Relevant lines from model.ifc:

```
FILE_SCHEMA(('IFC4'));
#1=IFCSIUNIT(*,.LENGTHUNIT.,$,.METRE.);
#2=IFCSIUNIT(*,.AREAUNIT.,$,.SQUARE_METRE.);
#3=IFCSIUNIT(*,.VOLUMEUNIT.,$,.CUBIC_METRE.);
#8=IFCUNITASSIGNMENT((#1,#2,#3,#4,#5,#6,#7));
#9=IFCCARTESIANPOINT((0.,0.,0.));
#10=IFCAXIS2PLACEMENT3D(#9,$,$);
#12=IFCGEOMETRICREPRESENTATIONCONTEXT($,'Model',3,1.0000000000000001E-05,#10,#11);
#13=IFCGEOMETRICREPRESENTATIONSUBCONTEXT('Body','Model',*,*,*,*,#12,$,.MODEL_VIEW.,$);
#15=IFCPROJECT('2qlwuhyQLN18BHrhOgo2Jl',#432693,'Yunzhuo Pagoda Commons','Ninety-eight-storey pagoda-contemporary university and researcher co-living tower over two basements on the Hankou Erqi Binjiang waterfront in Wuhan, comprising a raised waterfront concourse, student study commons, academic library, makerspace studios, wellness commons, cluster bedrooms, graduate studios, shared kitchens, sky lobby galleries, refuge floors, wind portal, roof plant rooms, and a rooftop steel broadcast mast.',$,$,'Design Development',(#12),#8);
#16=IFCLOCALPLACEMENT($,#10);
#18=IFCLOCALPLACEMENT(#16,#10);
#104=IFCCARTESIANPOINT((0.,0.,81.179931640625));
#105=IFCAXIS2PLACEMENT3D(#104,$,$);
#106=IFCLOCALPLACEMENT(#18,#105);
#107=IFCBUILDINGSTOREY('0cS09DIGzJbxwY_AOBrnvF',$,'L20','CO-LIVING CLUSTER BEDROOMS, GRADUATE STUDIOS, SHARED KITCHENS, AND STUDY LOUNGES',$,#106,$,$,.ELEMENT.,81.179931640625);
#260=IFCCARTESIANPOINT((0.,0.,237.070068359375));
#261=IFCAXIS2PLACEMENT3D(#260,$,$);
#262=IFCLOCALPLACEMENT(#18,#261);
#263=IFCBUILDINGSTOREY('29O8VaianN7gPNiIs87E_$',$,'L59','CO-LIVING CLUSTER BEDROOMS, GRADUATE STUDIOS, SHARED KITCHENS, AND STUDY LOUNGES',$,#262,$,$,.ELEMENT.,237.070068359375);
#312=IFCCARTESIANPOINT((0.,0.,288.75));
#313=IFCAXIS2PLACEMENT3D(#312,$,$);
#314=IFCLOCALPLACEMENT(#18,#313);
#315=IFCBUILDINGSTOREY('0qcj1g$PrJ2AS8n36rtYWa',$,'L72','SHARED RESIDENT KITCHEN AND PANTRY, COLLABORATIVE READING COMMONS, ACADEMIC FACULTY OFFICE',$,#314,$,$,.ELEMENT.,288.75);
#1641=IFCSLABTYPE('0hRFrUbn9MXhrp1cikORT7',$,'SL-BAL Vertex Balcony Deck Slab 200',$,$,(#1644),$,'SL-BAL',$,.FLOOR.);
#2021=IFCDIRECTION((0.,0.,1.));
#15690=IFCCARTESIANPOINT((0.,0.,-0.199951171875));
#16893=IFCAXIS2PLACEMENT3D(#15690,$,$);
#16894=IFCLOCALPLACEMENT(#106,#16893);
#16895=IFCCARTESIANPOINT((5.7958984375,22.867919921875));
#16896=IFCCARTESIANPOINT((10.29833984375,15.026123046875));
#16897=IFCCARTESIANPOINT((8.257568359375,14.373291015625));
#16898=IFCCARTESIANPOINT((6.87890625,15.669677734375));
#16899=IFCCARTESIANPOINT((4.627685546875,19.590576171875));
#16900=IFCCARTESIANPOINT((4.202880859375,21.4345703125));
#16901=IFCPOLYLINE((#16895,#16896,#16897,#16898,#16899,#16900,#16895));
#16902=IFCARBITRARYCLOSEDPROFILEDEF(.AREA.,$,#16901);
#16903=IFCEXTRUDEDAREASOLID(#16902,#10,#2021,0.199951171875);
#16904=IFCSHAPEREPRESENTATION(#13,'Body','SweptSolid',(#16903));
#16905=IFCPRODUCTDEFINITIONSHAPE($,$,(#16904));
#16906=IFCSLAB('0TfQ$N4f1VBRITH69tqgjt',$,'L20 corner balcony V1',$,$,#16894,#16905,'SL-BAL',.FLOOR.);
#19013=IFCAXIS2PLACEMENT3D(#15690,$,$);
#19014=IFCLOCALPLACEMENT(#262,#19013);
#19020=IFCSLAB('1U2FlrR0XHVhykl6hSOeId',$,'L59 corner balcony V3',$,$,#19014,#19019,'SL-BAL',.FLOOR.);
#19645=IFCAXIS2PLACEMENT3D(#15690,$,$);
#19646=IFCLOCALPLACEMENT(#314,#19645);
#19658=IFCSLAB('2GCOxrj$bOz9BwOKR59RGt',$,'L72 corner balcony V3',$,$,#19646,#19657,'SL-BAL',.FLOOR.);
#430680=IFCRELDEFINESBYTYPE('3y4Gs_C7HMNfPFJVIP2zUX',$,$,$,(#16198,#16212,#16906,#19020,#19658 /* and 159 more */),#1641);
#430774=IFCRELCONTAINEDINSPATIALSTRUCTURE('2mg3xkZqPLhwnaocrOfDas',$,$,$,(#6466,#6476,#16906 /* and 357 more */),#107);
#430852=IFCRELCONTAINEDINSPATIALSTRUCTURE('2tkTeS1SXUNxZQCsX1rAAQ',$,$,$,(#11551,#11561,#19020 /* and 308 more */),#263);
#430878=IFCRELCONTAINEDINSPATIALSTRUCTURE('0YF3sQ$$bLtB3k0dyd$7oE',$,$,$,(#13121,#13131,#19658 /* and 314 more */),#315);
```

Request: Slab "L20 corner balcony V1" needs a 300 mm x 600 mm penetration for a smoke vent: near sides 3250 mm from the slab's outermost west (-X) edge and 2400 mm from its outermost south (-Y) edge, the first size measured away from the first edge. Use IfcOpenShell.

```python
import numpy as np
import ifcopenshell
import ifcopenshell.api.feature
import ifcopenshell.api.geometry
import ifcopenshell.api.root
import ifcopenshell.geom
import ifcopenshell.util.placement
import ifcopenshell.util.representation
import ifcopenshell.util.shape
import ifcopenshell.util.unit

model = ifcopenshell.open("model.ifc")
unit_scale = ifcopenshell.util.unit.calculate_unit_scale(model)
settings = ifcopenshell.geom.settings()


def volume(element):
    """Net volume in cubic metres, openings subtracted."""
    shape = ifcopenshell.geom.create_shape(settings, element)
    return ifcopenshell.util.shape.get_volume(shape.geometry)


slab = model.by_guid("0TfQ$N4f1VBRITH69tqgjt")
before = volume(slab)

# Extent in the slab's own axes, in metres. The edges named are its -X and -Y sides.
slab_shape = ifcopenshell.geom.create_shape(settings, slab)
vertices = ifcopenshell.util.shape.get_vertices(slab_shape.geometry)
x_min, y_min, bottom = vertices.min(axis=0)
top = vertices[:, 2].max()

opening = ifcopenshell.api.root.create_entity(model, ifc_class="IfcOpeningElement", name="Smoke vent opening", predefined_type="OPENING")
context = ifcopenshell.util.representation.get_context(model, "Model", "Body", "MODEL_VIEW")
width, depth = 0.3, 0.6
outline = [(0.0, 0.0), (width, 0.0), (width, depth), (0.0, depth), (0.0, 0.0)]
# Overshoot both faces by 50 mm so the cut is clean.
shape = ifcopenshell.api.geometry.add_slab_representation(
    model, context=context, depth=top - bottom + 0.1, polyline=outline
)
ifcopenshell.api.geometry.assign_representation(model, product=opening, representation=shape)

matrix = ifcopenshell.util.placement.get_local_placement(slab.ObjectPlacement)
matrix[:, 3] = matrix @ np.append(np.array([x_min + 3.25, y_min + 2.4, bottom - 0.05]) / unit_scale, 1.0)
ifcopenshell.api.geometry.edit_object_placement(model, product=opening, matrix=matrix, is_si=False)
ifcopenshell.api.feature.add_feature(model, feature=opening, element=slab)

after = volume(slab)

print(f"slab volume {before:.3f} -> {after:.3f} m3")

model.write("model_v2.ifc")
```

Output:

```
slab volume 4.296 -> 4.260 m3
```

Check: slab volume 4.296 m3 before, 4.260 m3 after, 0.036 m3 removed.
